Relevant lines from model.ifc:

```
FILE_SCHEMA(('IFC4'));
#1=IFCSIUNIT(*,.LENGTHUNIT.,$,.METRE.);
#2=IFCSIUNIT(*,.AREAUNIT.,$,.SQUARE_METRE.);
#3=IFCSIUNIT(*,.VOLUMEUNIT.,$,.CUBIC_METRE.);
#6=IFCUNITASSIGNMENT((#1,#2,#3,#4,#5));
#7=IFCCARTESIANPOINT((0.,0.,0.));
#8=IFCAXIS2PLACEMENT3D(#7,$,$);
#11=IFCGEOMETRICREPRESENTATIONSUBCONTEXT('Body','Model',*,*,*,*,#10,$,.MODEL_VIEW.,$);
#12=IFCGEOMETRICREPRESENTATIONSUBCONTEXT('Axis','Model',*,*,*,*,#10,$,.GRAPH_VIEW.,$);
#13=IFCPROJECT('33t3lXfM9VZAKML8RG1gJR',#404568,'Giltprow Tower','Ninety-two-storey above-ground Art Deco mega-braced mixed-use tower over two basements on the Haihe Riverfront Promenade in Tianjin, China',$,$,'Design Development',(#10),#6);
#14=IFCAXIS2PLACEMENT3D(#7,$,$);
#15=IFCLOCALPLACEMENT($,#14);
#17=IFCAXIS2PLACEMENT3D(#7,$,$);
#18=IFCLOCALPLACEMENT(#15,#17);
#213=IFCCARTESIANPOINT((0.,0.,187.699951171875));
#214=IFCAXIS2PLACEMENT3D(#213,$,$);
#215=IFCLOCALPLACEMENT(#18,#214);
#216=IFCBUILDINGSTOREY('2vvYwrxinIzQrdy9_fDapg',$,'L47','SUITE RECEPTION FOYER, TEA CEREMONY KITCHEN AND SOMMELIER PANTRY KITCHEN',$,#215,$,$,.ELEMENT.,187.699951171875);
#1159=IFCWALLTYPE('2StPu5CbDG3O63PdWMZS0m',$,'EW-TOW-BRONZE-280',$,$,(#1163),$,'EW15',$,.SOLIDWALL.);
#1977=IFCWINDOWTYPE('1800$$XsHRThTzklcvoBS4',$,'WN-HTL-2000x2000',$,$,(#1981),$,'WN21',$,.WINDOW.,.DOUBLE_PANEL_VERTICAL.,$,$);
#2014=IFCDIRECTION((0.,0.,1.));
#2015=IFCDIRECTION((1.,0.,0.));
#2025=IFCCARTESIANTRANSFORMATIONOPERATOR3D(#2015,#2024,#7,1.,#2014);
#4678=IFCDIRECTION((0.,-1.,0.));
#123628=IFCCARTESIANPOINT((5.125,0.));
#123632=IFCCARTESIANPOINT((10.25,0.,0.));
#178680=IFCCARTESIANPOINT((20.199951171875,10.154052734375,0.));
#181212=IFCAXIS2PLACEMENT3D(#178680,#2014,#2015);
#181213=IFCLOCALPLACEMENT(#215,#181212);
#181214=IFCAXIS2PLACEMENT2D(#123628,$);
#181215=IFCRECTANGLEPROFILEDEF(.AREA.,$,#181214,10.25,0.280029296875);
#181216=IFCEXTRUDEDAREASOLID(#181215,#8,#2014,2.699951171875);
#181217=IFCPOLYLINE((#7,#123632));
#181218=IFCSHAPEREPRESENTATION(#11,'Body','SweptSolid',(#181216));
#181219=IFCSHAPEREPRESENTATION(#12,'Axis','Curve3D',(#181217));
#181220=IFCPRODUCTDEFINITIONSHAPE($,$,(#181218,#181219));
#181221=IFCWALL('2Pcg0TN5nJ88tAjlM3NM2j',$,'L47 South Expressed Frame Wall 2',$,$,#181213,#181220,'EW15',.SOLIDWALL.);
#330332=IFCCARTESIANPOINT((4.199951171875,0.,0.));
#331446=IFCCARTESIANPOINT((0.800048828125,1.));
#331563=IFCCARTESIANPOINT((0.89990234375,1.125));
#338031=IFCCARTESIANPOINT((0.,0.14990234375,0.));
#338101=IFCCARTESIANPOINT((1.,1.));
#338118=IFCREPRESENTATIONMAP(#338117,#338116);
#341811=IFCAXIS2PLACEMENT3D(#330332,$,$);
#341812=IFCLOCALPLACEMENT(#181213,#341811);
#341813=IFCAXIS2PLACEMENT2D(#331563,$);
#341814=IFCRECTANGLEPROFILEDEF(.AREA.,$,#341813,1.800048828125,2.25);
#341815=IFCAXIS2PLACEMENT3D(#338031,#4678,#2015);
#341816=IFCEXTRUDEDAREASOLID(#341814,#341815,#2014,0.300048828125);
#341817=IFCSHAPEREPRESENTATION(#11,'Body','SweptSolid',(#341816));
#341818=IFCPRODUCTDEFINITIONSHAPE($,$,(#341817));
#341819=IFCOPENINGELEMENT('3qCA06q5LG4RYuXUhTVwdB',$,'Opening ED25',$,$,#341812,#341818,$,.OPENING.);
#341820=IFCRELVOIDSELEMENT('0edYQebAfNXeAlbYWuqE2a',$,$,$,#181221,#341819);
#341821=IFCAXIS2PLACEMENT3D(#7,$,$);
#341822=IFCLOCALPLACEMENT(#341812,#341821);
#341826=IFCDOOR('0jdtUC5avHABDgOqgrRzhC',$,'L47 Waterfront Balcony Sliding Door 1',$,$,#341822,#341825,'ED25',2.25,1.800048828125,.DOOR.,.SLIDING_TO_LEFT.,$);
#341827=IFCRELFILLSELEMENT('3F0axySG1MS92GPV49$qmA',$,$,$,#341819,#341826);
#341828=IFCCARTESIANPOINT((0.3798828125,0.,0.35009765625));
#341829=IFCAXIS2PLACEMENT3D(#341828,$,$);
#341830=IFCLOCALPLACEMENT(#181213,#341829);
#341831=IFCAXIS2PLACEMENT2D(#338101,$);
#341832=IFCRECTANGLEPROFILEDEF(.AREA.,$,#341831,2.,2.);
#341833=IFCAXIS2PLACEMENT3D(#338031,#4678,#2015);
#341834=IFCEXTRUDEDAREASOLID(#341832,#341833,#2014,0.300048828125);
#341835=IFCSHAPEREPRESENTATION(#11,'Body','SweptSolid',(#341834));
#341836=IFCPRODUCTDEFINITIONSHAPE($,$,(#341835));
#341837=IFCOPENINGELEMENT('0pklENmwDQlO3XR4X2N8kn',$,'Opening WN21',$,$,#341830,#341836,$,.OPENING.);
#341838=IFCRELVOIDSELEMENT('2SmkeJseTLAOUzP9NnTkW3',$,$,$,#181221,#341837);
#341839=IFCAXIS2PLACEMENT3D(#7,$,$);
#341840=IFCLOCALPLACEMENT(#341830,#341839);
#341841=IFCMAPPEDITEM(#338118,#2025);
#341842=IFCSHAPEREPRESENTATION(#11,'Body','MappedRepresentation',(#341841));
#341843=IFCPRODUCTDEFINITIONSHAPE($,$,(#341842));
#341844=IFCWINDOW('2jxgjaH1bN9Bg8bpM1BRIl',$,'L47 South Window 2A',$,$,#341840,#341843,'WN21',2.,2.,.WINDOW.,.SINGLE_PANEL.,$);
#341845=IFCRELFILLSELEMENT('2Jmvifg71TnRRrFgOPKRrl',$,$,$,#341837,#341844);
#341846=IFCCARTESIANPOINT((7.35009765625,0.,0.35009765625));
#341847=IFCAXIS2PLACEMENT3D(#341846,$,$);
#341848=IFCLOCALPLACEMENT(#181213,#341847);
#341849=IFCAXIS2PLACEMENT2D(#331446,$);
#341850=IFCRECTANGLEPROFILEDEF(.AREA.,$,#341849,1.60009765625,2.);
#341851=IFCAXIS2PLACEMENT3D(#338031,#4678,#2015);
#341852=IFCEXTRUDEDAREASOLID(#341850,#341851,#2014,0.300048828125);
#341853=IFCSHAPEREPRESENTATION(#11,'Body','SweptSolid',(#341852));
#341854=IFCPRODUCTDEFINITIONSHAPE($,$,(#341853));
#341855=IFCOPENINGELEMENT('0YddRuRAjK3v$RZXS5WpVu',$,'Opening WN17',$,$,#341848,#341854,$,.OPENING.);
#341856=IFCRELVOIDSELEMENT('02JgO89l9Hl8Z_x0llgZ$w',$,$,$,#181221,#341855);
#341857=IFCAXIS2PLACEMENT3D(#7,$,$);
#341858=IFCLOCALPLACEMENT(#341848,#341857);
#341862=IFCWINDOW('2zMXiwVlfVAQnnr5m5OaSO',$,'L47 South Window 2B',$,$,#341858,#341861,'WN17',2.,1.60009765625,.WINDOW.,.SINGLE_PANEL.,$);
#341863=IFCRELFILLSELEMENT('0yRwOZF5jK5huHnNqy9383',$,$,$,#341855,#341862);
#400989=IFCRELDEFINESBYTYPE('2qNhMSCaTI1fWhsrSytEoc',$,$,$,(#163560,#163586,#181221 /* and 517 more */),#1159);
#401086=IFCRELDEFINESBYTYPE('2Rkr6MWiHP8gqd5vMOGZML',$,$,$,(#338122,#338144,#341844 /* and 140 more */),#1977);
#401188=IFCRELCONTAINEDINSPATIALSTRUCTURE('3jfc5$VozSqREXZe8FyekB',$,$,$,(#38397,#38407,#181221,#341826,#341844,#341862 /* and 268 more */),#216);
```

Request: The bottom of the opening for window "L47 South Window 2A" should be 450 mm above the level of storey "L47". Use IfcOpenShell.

```python
import numpy as np
import ifcopenshell
import ifcopenshell.api.geometry
import ifcopenshell.geom
import ifcopenshell.util.element
import ifcopenshell.util.placement
import ifcopenshell.util.shape
import ifcopenshell.util.unit

model = ifcopenshell.open("model.ifc")
unit_scale = ifcopenshell.util.unit.calculate_unit_scale(model)

window = model.by_guid("2jxgjaH1bN9Bg8bpM1BRIl")
opening = window.FillsVoids[0].RelatingOpeningElement
storey = ifcopenshell.util.element.get_container(window, ifc_class="IfcBuildingStorey")
level = ifcopenshell.util.placement.get_local_placement(storey.ObjectPlacement)[2, 3]

# The opening's origin need not be at the sill, so measure its lowest point.
shape = ifcopenshell.geom.create_shape(ifcopenshell.geom.settings(), opening)
bottom = ifcopenshell.util.shape.get_shape_bottom_elevation(shape, shape.geometry) / unit_scale
dz = level + 0.45 / unit_scale - bottom

shift = np.array([0.0, 0.0, dz])
# The window is placed relative to its opening, so it follows when the opening moves.
matrix = ifcopenshell.util.placement.get_local_placement(opening.ObjectPlacement)
matrix[:3, 3] += shift
ifcopenshell.api.geometry.edit_object_placement(
    model, product=opening, matrix=matrix, is_si=False, should_transform_children=True
)

print(f"moved by {dz * unit_scale:+.3f} m")

model.write("model_edited.ifc")
```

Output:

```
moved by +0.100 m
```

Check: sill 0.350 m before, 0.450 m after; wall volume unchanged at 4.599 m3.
